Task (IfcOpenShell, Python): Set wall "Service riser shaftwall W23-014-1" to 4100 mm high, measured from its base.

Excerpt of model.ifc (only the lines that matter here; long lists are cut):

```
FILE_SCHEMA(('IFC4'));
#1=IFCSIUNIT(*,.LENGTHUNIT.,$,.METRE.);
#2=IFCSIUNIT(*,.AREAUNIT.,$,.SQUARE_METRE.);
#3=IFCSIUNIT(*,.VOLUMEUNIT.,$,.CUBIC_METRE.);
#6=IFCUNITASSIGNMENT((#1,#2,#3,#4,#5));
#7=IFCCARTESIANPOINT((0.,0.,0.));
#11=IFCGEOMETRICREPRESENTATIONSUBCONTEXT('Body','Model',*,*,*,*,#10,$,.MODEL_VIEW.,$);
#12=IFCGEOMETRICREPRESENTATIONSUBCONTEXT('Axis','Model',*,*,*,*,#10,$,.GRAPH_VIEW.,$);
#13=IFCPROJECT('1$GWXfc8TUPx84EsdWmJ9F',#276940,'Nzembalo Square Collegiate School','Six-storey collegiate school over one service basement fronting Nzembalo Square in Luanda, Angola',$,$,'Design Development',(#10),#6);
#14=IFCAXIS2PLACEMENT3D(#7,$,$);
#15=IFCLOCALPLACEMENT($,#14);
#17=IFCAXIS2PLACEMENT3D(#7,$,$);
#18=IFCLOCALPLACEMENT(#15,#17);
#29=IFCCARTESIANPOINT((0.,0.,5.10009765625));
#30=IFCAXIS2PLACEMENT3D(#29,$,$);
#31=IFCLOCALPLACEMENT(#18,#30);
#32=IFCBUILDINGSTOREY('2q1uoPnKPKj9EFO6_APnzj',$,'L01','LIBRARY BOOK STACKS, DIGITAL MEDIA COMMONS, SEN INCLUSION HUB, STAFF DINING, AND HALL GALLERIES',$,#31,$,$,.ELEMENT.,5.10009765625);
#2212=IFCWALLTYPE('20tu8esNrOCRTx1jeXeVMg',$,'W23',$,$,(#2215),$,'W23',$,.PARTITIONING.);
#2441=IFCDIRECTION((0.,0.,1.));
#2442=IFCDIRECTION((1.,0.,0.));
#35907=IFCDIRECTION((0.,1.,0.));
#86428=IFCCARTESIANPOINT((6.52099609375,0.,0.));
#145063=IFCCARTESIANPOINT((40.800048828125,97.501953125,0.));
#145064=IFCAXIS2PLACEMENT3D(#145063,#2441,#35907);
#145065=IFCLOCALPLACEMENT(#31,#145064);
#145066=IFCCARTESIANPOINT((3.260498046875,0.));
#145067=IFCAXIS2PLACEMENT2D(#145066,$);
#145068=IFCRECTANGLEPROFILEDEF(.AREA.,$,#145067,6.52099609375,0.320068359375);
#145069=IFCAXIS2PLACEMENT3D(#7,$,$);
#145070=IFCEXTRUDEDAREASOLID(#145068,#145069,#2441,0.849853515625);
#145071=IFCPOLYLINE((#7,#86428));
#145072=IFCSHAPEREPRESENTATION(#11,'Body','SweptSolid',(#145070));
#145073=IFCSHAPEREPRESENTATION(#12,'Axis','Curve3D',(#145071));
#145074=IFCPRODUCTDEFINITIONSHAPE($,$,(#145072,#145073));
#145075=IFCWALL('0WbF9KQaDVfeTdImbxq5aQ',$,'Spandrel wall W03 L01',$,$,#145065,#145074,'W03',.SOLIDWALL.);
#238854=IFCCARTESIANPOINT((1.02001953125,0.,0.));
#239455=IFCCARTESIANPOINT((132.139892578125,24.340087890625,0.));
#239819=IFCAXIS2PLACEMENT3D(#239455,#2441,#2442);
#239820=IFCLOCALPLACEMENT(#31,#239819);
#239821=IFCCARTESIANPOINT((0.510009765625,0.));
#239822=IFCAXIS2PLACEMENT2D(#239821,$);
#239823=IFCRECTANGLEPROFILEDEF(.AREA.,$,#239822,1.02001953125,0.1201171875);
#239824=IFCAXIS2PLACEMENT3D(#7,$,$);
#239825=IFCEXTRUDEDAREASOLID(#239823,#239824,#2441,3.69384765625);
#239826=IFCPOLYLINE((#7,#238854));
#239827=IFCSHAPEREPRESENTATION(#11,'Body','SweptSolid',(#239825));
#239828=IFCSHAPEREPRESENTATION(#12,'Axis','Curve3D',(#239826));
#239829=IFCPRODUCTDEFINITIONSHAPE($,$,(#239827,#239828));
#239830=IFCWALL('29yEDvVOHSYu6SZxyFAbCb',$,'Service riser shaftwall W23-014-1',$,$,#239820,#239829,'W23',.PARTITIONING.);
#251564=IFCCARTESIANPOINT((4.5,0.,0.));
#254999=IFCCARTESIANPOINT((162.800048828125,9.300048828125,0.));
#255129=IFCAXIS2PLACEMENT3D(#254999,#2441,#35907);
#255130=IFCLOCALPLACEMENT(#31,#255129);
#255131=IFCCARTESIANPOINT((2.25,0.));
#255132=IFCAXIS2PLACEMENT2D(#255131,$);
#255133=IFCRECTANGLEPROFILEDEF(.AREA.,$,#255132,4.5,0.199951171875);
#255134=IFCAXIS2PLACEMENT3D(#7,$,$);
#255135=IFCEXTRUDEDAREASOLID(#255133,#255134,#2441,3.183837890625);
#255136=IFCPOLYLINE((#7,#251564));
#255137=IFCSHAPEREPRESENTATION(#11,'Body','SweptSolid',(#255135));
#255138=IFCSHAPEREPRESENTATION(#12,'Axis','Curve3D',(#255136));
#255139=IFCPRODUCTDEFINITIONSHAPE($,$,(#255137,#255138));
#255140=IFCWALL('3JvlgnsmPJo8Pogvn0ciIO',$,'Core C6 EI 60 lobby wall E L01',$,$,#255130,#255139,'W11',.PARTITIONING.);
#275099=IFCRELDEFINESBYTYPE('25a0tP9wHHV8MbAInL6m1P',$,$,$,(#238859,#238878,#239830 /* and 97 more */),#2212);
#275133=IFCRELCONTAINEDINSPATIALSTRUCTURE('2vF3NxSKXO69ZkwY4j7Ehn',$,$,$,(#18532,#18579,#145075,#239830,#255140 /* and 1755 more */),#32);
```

```python
import ifcopenshell
import ifcopenshell.geom
import ifcopenshell.util.representation
import ifcopenshell.util.shape

model = ifcopenshell.open("model.ifc")
settings = ifcopenshell.geom.settings()


def volume(element):
    """Net volume in cubic metres, openings subtracted."""
    shape = ifcopenshell.geom.create_shape(settings, element)
    return ifcopenshell.util.shape.get_volume(shape.geometry)


wall = model.by_guid("29yEDvVOHSYu6SZxyFAbCb")
before = volume(wall)

body = ifcopenshell.util.representation.get_representation(wall, "Model", "Body")
solid = body.Items[0]
old_height = solid.Depth
solid.Depth = 4.1
after = volume(wall)

print(f"height {old_height:g} -> {solid.Depth:g}, volume {before:.3f} -> {after:.3f} m3")

model.write("model_rev.ifc")
```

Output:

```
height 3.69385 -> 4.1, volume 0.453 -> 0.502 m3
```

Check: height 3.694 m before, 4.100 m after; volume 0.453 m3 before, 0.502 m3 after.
